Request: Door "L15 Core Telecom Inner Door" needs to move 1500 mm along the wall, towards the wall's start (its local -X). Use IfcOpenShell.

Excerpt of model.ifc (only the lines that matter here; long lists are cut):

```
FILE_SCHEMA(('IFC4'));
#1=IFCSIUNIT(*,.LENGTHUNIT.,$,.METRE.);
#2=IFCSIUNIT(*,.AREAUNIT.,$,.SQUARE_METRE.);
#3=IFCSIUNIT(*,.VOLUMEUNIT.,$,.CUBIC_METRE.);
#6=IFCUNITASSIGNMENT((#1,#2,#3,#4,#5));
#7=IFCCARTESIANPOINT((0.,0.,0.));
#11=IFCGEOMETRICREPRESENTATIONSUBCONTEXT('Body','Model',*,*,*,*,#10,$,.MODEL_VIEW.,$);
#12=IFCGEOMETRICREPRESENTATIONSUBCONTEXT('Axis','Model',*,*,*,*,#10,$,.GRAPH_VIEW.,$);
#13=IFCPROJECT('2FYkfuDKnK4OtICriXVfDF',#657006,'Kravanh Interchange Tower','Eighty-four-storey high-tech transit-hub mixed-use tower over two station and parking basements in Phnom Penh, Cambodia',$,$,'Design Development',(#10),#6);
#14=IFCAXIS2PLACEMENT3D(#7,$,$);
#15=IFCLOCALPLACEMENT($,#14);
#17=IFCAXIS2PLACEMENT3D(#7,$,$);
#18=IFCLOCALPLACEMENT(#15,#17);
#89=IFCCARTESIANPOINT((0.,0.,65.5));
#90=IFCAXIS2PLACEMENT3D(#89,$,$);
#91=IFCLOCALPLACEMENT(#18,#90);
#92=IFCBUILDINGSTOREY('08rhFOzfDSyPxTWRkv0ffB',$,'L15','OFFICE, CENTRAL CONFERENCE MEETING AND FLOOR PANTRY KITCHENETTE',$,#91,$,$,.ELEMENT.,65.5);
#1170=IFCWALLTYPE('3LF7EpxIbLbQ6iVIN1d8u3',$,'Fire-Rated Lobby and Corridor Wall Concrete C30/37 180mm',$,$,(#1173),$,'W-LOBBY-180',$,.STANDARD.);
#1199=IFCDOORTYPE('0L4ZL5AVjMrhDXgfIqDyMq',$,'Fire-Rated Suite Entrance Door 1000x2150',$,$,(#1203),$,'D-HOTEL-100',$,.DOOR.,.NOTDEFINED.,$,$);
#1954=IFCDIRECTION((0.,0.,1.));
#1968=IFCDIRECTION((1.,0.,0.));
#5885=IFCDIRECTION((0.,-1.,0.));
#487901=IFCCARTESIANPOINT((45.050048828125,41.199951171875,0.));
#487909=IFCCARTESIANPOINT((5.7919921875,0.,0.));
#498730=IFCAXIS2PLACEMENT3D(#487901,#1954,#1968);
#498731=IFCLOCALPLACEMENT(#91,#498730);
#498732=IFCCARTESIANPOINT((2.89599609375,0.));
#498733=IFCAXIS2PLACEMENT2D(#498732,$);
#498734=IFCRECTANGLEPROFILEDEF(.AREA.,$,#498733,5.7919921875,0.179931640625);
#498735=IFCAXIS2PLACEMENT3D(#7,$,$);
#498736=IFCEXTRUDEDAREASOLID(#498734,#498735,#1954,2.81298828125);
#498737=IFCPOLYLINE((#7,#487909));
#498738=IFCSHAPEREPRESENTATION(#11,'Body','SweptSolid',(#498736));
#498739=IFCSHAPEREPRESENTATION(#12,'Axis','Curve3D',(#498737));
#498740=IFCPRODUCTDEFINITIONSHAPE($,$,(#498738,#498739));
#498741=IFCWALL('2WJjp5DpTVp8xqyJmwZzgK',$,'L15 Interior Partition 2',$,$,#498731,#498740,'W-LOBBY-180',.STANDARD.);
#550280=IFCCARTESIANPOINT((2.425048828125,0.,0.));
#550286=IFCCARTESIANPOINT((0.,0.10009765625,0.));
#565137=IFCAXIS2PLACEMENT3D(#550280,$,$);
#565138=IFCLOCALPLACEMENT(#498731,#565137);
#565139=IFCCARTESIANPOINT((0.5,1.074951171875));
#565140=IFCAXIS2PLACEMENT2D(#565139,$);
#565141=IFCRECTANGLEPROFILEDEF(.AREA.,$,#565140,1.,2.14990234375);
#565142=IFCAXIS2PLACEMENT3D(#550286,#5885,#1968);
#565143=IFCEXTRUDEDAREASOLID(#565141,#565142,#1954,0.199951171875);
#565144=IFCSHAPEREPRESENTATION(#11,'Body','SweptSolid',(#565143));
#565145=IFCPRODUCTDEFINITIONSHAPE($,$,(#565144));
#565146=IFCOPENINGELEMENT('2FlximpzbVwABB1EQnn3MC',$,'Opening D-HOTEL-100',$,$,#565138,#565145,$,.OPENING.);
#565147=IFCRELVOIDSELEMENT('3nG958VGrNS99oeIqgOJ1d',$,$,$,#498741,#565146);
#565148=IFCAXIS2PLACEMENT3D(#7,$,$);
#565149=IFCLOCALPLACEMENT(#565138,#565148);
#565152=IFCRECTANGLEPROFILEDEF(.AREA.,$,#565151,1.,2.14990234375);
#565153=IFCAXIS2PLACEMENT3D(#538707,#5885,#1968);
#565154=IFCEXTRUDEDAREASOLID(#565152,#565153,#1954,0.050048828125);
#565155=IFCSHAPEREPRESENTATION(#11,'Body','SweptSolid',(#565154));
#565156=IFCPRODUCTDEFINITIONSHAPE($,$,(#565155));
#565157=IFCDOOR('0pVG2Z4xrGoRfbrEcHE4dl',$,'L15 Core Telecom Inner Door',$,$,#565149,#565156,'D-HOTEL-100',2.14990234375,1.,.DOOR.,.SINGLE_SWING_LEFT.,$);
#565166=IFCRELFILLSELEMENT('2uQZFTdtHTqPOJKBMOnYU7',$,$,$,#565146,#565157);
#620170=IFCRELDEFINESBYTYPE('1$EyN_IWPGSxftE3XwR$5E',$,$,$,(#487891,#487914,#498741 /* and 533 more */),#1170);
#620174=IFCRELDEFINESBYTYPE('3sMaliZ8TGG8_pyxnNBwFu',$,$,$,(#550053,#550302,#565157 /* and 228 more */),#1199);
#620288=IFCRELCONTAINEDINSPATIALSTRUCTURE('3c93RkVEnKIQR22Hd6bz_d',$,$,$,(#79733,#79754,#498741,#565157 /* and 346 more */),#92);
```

```python
import ifcopenshell
import ifcopenshell.api.geometry
import ifcopenshell.util.placement
import ifcopenshell.util.unit

model = ifcopenshell.open("model.ifc")
unit_scale = ifcopenshell.util.unit.calculate_unit_scale(model)

door = model.by_id(565157)
opening = door.FillsVoids[0].RelatingOpeningElement
wall = opening.VoidsElements[0].RelatingBuildingElement

wall_matrix = ifcopenshell.util.placement.get_local_placement(wall.ObjectPlacement)
shift = wall_matrix[:3, 0] * -1.5 / unit_scale
before = ifcopenshell.util.placement.get_local_placement(door.ObjectPlacement)[:3, 3].copy()

# The door is placed relative to its opening, so it follows when the opening moves.
matrix = ifcopenshell.util.placement.get_local_placement(opening.ObjectPlacement)
matrix[:3, 3] += shift
ifcopenshell.api.geometry.edit_object_placement(
    model, product=opening, matrix=matrix, is_si=False, should_transform_children=True
)

after = ifcopenshell.util.placement.get_local_placement(door.ObjectPlacement)[:3, 3]
print("door moved by", (after - before).round(3) + 0.0)

model.write("model_rev.ifc")
```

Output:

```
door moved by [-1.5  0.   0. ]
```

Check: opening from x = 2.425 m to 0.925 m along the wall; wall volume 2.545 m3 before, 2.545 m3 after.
